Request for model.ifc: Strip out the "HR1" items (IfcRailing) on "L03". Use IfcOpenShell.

First a look at what the model holds.

```python
import ifcopenshell
import ifcopenshell.util.element

model = ifcopenshell.open("model.ifc")
print(model.schema)
storey = next(s for s in model.by_type("IfcBuildingStorey") if s.Name == "L03")
railings = [e for e in ifcopenshell.util.element.get_decomposition(storey) if e.is_a("IfcRailing")]
seen = {}
for e in railings:
    element_type = ifcopenshell.util.element.get_type(e)
    name = element_type.Name if element_type not in (None, e) else None
    seen[name] = seen.get(name, 0) + 1
for name, count in sorted(seen.items(), key=str):
    print(count, "x", name)
```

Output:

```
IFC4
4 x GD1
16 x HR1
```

```python
import ifcopenshell
import ifcopenshell.api.root
import ifcopenshell.util.element

model = ifcopenshell.open("model.ifc")

storey = next(s for s in model.by_type("IfcBuildingStorey") if s.Name == "L03")
railings = [e for e in ifcopenshell.util.element.get_decomposition(storey) if e.is_a("IfcRailing")]
targets = [e for e in railings if (t := ifcopenshell.util.element.get_type(e)) not in (None, e) and t.Name == "HR1"]

for e in targets:
    ifcopenshell.api.root.remove_product(model, product=e)
print(len(targets), "removed")

model.write("model_updated.ifc")
```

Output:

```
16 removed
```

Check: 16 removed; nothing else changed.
